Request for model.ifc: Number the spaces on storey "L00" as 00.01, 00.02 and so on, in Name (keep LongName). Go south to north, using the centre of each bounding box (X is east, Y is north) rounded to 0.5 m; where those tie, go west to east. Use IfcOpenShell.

First a look at what the model holds.

```python
import ifcopenshell
import ifcopenshell.util.element
import ifcopenshell.util.placement

model = ifcopenshell.open("model.ifc")
print(model.schema)
storey = next(s for s in model.by_type("IfcBuildingStorey") if s.Name == "L00")
spaces = [e for e in ifcopenshell.util.element.get_decomposition(storey) if e.is_a("IfcSpace")]
for e in sorted(spaces, key=lambda e: e.id()):
    origin = ifcopenshell.util.placement.get_local_placement(e.ObjectPlacement)[:3, 3]
    print(e.id(), e.Name, e.LongName, origin.round(2) + 0.0, sep=" | ")
```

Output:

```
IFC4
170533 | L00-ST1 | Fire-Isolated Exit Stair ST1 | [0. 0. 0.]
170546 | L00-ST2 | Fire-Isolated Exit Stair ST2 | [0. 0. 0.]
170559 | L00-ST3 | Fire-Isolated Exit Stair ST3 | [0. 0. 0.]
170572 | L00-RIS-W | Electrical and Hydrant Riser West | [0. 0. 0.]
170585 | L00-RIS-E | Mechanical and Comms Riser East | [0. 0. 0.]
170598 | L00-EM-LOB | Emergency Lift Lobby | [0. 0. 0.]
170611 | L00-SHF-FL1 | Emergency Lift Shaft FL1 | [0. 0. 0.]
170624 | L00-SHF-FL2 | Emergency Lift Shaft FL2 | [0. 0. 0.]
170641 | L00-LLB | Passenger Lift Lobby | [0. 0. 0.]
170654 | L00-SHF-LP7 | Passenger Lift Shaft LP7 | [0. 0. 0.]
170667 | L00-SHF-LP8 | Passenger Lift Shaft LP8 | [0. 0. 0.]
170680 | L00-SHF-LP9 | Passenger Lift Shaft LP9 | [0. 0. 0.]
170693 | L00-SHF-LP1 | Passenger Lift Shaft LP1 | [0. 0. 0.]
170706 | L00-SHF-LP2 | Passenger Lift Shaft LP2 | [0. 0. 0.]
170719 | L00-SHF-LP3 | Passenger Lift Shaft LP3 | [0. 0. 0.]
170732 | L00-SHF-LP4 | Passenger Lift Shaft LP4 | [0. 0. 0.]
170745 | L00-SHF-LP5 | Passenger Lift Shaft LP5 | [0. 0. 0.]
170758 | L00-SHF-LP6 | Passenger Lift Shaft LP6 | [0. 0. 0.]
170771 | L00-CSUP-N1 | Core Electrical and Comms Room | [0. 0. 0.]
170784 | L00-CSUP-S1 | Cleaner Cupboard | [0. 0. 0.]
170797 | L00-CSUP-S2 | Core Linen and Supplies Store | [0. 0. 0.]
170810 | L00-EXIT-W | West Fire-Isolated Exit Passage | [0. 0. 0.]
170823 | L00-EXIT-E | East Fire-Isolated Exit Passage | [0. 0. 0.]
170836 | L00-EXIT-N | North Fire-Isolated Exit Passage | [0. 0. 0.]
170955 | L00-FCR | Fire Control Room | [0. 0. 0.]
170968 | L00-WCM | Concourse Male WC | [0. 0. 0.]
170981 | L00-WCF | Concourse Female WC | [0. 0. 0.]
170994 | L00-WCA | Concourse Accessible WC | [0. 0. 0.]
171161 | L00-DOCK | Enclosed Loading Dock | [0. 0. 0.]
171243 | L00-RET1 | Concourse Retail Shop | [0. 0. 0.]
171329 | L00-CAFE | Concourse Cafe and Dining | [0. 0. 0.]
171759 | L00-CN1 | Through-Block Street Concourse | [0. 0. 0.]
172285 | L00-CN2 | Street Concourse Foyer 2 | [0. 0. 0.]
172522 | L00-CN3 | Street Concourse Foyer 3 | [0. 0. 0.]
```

```python
import ifcopenshell
import ifcopenshell.geom
import ifcopenshell.util.element
import ifcopenshell.util.shape

model = ifcopenshell.open("model.ifc")
settings = ifcopenshell.geom.settings()
settings.set("use-world-coords", True)


def centre(element):
    shape = ifcopenshell.geom.create_shape(settings, element)
    return ifcopenshell.util.shape.get_bbox_centroid(shape.geometry)


storey = next(s for s in model.by_type("IfcBuildingStorey") if s.Name == "L00")
spaces = [e for e in ifcopenshell.util.element.get_decomposition(storey) if e.is_a("IfcSpace")]

# Insertion points can sit at a corner or the storey origin, so sort by the geometry (in metres).
centres = {e: centre(e) for e in spaces}
spaces.sort(key=lambda e: (round(centres[e][1] / 0.5), centres[e][0]))

for i, e in enumerate(spaces, start=1):
    number = f"00.{i:02d}"
    e.Name = number
    print(e.id(), number)

model.write("model_updated.ifc")
```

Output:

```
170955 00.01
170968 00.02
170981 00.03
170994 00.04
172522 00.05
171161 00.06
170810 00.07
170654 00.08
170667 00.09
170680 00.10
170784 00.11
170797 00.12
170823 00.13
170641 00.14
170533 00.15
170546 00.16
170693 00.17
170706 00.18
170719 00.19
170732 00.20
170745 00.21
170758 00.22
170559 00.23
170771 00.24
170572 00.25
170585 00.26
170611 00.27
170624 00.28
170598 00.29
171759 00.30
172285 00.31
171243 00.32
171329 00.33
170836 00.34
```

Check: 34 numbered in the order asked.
